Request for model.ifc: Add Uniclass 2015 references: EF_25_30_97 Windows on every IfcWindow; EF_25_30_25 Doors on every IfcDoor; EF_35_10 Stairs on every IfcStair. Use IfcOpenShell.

First a look at what the model holds.

```python
import ifcopenshell

model = ifcopenshell.open("model.ifc")
print(model.schema)
print("classifications:", [c.Name for c in model.by_type("IfcClassification")])
for ifc_class in ("IfcDoor", "IfcRoof", "IfcStair", "IfcWall", "IfcWindow"):
    print(ifc_class, len(model.by_type(ifc_class)))
```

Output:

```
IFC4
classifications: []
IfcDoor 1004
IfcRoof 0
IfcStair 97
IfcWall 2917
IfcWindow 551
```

```python
import ifcopenshell
import ifcopenshell.api.classification

model = ifcopenshell.open("model.ifc")

system = ifcopenshell.api.classification.add_classification(model, classification="Uniclass 2015")

codes = {
    "IfcWindow": ("EF_25_30_97", "Windows"),
    "IfcDoor": ("EF_25_30_25", "Doors"),
    "IfcStair": ("EF_35_10", "Stairs"),
}
for ifc_class, (code, name) in codes.items():
    products = model.by_type(ifc_class)
    ifcopenshell.api.classification.add_reference(
        model, products=products, classification=system, identification=code, name=name
    )
    print(code, len(products))

model.write("model_updated.ifc")
```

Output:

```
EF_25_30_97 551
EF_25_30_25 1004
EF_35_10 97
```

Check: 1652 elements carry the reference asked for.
